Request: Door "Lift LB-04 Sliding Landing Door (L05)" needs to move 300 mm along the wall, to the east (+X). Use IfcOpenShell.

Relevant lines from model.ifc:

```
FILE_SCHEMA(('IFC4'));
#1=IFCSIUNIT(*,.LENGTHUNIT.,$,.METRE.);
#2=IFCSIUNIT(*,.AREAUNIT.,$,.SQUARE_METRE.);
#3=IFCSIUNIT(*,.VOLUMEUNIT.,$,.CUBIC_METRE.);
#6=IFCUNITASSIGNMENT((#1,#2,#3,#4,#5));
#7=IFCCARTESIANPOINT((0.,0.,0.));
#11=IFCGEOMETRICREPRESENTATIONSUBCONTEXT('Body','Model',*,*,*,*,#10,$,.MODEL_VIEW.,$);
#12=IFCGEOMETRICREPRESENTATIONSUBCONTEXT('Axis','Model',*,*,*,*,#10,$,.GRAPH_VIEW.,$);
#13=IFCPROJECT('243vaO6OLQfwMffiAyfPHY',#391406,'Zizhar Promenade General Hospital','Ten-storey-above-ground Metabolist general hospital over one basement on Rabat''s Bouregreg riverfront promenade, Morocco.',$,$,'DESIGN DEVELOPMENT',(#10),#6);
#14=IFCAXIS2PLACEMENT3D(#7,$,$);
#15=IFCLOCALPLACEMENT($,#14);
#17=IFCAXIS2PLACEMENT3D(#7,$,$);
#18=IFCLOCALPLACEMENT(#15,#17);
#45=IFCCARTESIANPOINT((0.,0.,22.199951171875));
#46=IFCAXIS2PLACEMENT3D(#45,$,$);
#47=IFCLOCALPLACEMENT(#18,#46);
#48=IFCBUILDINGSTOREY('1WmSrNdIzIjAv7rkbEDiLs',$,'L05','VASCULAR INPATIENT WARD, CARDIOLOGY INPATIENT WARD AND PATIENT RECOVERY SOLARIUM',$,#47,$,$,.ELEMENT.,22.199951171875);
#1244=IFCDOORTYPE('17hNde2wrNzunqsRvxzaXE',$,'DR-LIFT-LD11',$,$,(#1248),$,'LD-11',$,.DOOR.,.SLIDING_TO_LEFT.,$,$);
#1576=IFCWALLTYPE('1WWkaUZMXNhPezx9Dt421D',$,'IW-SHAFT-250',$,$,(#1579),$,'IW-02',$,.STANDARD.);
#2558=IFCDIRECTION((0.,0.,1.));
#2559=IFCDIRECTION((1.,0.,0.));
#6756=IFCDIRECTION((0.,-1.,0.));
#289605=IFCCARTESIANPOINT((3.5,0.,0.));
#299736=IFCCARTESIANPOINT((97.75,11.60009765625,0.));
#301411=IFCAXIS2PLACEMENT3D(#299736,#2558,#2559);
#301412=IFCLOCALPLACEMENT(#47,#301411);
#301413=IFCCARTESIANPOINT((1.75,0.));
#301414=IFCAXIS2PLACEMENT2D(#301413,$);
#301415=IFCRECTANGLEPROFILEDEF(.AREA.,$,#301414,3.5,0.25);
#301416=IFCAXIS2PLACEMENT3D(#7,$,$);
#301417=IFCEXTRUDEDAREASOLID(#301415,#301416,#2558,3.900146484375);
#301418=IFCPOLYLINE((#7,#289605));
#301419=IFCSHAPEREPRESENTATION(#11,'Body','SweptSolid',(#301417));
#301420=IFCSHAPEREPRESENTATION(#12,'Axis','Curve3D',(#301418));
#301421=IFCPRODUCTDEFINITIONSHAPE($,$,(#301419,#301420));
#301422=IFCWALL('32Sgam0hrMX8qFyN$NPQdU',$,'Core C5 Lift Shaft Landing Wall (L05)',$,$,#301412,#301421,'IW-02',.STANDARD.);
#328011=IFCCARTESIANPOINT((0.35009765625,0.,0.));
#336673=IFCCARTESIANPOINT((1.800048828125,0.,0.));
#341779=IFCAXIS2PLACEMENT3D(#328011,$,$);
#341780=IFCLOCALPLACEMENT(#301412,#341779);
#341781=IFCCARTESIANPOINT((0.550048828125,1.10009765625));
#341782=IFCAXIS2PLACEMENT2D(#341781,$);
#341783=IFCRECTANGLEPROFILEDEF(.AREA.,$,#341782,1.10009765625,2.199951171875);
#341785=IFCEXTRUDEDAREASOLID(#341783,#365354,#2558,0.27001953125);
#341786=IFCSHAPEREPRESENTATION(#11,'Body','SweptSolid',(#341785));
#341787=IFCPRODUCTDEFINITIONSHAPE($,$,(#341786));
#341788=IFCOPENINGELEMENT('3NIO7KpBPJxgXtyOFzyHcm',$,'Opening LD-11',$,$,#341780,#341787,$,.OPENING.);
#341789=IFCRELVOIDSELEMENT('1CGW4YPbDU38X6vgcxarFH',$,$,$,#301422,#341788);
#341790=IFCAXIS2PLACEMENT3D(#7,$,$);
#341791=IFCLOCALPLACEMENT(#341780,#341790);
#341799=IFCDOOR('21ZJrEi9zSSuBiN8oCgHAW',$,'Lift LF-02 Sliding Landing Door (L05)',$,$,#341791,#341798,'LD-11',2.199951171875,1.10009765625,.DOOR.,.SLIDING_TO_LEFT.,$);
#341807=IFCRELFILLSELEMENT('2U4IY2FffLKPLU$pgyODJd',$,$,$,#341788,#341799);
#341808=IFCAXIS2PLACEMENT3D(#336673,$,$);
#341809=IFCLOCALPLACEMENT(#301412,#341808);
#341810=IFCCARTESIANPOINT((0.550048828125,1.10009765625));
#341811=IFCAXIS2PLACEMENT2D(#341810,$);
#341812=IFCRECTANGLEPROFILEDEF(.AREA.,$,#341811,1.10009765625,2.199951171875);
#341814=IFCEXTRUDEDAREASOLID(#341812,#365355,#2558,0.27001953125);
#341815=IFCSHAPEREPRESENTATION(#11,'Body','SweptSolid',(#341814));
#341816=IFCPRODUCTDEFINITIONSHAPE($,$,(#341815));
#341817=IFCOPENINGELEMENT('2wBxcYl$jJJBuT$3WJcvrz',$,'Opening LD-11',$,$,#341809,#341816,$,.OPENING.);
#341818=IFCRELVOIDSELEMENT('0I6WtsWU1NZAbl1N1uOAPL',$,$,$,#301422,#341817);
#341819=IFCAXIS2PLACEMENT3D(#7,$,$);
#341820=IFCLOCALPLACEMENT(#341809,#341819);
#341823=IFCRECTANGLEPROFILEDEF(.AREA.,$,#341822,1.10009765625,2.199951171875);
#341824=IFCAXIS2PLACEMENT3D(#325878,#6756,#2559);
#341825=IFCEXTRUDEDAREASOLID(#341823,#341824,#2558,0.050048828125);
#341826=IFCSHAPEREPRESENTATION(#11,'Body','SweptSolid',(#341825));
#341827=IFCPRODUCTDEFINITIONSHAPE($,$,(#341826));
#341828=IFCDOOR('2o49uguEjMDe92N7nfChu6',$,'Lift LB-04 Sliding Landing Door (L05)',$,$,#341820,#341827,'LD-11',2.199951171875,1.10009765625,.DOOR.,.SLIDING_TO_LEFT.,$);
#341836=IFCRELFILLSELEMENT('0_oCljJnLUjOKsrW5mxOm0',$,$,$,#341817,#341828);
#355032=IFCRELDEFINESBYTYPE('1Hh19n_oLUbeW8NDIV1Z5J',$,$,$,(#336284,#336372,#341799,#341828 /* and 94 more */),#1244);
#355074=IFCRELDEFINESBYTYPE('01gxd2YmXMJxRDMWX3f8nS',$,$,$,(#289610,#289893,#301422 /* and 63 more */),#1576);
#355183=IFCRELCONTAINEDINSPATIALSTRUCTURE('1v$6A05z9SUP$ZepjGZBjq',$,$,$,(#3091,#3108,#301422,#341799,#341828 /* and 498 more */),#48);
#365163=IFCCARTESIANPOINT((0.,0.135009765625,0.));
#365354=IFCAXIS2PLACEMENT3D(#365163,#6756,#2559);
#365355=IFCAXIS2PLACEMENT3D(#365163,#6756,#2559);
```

```python
import ifcopenshell
import ifcopenshell.api.geometry
import ifcopenshell.util.placement
import ifcopenshell.util.unit

model = ifcopenshell.open("model.ifc")
unit_scale = ifcopenshell.util.unit.calculate_unit_scale(model)

door = model.by_id(341828)
opening = door.FillsVoids[0].RelatingOpeningElement
wall = opening.VoidsElements[0].RelatingBuildingElement

wall_matrix = ifcopenshell.util.placement.get_local_placement(wall.ObjectPlacement)
shift = wall_matrix[:3, 0] * 0.3 / unit_scale
before = ifcopenshell.util.placement.get_local_placement(door.ObjectPlacement)[:3, 3].copy()

# The door is placed relative to its opening, so it follows when the opening moves.
matrix = ifcopenshell.util.placement.get_local_placement(opening.ObjectPlacement)
matrix[:3, 3] += shift
ifcopenshell.api.geometry.edit_object_placement(
    model, product=opening, matrix=matrix, is_si=False, should_transform_children=True
)

after = ifcopenshell.util.placement.get_local_placement(door.ObjectPlacement)[:3, 3]
print("door moved by", (after - before).round(3) + 0.0)

model.write("model_rev.ifc")
```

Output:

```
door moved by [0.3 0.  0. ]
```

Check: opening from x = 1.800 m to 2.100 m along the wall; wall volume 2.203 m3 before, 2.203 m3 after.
